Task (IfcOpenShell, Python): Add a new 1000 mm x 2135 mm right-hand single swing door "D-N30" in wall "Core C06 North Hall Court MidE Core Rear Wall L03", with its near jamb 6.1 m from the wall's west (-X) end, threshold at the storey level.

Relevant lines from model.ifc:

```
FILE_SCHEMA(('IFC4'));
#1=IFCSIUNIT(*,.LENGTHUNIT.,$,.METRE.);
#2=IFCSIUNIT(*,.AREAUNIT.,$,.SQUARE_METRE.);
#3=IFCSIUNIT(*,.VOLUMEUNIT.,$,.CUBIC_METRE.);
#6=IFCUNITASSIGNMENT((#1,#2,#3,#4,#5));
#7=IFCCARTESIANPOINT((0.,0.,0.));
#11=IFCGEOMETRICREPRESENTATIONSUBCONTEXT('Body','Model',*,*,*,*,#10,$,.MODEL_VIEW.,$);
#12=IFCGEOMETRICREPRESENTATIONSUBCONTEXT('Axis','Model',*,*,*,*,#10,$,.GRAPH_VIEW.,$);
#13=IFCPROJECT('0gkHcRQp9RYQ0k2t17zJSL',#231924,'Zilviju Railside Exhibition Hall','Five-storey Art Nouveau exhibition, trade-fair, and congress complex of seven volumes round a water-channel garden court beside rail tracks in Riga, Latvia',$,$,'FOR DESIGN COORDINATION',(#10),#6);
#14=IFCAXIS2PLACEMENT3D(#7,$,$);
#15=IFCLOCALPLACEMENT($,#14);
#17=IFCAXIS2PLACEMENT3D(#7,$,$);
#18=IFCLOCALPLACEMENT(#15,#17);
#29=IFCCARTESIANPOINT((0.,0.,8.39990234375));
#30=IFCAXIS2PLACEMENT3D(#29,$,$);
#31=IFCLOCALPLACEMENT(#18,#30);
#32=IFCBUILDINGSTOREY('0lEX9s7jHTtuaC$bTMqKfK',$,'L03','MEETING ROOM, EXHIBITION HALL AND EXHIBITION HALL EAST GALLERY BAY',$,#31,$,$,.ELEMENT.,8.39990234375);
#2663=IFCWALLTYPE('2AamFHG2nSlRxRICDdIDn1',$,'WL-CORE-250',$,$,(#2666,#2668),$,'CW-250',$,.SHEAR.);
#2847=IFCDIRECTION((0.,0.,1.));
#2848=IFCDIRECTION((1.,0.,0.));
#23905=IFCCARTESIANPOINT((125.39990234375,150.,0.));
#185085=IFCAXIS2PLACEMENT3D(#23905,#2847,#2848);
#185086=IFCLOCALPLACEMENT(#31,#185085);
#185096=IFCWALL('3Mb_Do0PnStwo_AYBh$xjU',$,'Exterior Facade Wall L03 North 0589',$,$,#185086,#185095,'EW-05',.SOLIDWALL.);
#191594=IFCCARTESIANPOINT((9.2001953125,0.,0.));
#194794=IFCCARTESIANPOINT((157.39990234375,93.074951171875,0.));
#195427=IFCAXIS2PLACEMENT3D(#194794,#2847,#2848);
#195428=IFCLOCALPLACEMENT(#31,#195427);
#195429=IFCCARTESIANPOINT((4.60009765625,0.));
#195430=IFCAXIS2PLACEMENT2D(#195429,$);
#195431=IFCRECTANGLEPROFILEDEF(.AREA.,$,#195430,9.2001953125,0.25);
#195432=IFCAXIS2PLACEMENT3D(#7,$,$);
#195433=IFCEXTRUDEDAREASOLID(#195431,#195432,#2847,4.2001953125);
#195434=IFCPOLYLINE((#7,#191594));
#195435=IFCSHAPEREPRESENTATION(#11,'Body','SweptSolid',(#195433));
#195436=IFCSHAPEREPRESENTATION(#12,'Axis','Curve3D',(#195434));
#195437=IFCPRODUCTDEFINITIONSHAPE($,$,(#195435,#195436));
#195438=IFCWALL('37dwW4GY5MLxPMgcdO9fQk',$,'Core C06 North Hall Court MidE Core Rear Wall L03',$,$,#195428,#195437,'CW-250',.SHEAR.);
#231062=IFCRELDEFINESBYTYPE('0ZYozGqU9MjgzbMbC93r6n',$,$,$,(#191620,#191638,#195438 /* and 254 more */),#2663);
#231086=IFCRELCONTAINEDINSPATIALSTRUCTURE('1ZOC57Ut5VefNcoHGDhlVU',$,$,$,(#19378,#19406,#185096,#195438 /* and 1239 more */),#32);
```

```python
import numpy as np
import ifcopenshell
import ifcopenshell.api.feature
import ifcopenshell.api.geometry
import ifcopenshell.api.root
import ifcopenshell.api.spatial
import ifcopenshell.geom
import ifcopenshell.util.element
import ifcopenshell.util.placement
import ifcopenshell.util.representation
import ifcopenshell.util.shape
import ifcopenshell.util.unit

model = ifcopenshell.open("model.ifc")
unit_scale = ifcopenshell.util.unit.calculate_unit_scale(model)
settings = ifcopenshell.geom.settings()


def volume(element):
    """Net volume in cubic metres, openings subtracted."""
    shape = ifcopenshell.geom.create_shape(settings, element)
    return ifcopenshell.util.shape.get_volume(shape.geometry)


wall = model.by_id(195438)
storey = ifcopenshell.util.element.get_container(wall, ifc_class="IfcBuildingStorey")
context = ifcopenshell.util.representation.get_context(model, "Model", "Body", "MODEL_VIEW")
before = volume(wall)

width, height, from_end, sill = 1, 2.135, 6.1, 0.0  # metres

# The wall runs along its own X axis, and the end named is its -X end.
wall_shape = ifcopenshell.geom.create_shape(settings, wall)
x, y, z = ifcopenshell.util.shape.get_vertices(wall_shape.geometry).T
start = x.min() + from_end
face, thickness = float(y.min()), float(y.max() - y.min())
wall_matrix = ifcopenshell.util.placement.get_local_placement(wall.ObjectPlacement)
level = ifcopenshell.util.placement.get_local_placement(storey.ObjectPlacement)[2, 3]


def in_wall(x, y):
    """Placement at x, y metres in the wall's axes, at sill height."""
    matrix = wall_matrix.copy()
    matrix[:, 3] = wall_matrix @ np.array([x / unit_scale, y / unit_scale, 0.0, 1.0])
    matrix[2, 3] = level + sill / unit_scale
    return matrix


# Opening: a box that overshoots both wall faces by 50 mm.
opening = ifcopenshell.api.root.create_entity(model, ifc_class="IfcOpeningElement", predefined_type="OPENING")
box = ifcopenshell.api.geometry.add_wall_representation(
    model, context=context, length=width, height=height, thickness=thickness + 0.1
)
ifcopenshell.api.geometry.assign_representation(model, product=opening, representation=box)
ifcopenshell.api.geometry.edit_object_placement(model, product=opening, matrix=in_wall(start, face - 0.05), is_si=False)
ifcopenshell.api.feature.add_feature(model, feature=opening, element=wall)

door = ifcopenshell.api.root.create_entity(model, ifc_class="IfcDoor", name="D-N30", predefined_type="DOOR")
door.OverallWidth, door.OverallHeight = width / unit_scale, height / unit_scale
door.OperationType = "SINGLE_SWING_RIGHT"
body = ifcopenshell.api.geometry.add_door_representation(
    model,
    context=context,
    overall_width=door.OverallWidth,
    overall_height=door.OverallHeight,
    operation_type="SINGLE_SWING_RIGHT",
    lining_properties={"LiningDepth": thickness / unit_scale, "ThresholdDepth": thickness / unit_scale},
)
ifcopenshell.api.geometry.assign_representation(model, product=door, representation=body)
ifcopenshell.api.spatial.assign_container(model, products=[door], relating_structure=storey)
ifcopenshell.api.feature.add_filling(model, opening=opening, element=door)

# The lining spans the wall, so the door starts at the wall face.
ifcopenshell.api.geometry.edit_object_placement(model, product=door, matrix=in_wall(start, face), is_si=False)

after = volume(wall)

print(f"wall volume {before:.3f} -> {after:.3f} m3")

model.write("model_updated.ifc")
```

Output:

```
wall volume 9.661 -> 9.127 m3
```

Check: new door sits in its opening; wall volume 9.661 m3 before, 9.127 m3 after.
